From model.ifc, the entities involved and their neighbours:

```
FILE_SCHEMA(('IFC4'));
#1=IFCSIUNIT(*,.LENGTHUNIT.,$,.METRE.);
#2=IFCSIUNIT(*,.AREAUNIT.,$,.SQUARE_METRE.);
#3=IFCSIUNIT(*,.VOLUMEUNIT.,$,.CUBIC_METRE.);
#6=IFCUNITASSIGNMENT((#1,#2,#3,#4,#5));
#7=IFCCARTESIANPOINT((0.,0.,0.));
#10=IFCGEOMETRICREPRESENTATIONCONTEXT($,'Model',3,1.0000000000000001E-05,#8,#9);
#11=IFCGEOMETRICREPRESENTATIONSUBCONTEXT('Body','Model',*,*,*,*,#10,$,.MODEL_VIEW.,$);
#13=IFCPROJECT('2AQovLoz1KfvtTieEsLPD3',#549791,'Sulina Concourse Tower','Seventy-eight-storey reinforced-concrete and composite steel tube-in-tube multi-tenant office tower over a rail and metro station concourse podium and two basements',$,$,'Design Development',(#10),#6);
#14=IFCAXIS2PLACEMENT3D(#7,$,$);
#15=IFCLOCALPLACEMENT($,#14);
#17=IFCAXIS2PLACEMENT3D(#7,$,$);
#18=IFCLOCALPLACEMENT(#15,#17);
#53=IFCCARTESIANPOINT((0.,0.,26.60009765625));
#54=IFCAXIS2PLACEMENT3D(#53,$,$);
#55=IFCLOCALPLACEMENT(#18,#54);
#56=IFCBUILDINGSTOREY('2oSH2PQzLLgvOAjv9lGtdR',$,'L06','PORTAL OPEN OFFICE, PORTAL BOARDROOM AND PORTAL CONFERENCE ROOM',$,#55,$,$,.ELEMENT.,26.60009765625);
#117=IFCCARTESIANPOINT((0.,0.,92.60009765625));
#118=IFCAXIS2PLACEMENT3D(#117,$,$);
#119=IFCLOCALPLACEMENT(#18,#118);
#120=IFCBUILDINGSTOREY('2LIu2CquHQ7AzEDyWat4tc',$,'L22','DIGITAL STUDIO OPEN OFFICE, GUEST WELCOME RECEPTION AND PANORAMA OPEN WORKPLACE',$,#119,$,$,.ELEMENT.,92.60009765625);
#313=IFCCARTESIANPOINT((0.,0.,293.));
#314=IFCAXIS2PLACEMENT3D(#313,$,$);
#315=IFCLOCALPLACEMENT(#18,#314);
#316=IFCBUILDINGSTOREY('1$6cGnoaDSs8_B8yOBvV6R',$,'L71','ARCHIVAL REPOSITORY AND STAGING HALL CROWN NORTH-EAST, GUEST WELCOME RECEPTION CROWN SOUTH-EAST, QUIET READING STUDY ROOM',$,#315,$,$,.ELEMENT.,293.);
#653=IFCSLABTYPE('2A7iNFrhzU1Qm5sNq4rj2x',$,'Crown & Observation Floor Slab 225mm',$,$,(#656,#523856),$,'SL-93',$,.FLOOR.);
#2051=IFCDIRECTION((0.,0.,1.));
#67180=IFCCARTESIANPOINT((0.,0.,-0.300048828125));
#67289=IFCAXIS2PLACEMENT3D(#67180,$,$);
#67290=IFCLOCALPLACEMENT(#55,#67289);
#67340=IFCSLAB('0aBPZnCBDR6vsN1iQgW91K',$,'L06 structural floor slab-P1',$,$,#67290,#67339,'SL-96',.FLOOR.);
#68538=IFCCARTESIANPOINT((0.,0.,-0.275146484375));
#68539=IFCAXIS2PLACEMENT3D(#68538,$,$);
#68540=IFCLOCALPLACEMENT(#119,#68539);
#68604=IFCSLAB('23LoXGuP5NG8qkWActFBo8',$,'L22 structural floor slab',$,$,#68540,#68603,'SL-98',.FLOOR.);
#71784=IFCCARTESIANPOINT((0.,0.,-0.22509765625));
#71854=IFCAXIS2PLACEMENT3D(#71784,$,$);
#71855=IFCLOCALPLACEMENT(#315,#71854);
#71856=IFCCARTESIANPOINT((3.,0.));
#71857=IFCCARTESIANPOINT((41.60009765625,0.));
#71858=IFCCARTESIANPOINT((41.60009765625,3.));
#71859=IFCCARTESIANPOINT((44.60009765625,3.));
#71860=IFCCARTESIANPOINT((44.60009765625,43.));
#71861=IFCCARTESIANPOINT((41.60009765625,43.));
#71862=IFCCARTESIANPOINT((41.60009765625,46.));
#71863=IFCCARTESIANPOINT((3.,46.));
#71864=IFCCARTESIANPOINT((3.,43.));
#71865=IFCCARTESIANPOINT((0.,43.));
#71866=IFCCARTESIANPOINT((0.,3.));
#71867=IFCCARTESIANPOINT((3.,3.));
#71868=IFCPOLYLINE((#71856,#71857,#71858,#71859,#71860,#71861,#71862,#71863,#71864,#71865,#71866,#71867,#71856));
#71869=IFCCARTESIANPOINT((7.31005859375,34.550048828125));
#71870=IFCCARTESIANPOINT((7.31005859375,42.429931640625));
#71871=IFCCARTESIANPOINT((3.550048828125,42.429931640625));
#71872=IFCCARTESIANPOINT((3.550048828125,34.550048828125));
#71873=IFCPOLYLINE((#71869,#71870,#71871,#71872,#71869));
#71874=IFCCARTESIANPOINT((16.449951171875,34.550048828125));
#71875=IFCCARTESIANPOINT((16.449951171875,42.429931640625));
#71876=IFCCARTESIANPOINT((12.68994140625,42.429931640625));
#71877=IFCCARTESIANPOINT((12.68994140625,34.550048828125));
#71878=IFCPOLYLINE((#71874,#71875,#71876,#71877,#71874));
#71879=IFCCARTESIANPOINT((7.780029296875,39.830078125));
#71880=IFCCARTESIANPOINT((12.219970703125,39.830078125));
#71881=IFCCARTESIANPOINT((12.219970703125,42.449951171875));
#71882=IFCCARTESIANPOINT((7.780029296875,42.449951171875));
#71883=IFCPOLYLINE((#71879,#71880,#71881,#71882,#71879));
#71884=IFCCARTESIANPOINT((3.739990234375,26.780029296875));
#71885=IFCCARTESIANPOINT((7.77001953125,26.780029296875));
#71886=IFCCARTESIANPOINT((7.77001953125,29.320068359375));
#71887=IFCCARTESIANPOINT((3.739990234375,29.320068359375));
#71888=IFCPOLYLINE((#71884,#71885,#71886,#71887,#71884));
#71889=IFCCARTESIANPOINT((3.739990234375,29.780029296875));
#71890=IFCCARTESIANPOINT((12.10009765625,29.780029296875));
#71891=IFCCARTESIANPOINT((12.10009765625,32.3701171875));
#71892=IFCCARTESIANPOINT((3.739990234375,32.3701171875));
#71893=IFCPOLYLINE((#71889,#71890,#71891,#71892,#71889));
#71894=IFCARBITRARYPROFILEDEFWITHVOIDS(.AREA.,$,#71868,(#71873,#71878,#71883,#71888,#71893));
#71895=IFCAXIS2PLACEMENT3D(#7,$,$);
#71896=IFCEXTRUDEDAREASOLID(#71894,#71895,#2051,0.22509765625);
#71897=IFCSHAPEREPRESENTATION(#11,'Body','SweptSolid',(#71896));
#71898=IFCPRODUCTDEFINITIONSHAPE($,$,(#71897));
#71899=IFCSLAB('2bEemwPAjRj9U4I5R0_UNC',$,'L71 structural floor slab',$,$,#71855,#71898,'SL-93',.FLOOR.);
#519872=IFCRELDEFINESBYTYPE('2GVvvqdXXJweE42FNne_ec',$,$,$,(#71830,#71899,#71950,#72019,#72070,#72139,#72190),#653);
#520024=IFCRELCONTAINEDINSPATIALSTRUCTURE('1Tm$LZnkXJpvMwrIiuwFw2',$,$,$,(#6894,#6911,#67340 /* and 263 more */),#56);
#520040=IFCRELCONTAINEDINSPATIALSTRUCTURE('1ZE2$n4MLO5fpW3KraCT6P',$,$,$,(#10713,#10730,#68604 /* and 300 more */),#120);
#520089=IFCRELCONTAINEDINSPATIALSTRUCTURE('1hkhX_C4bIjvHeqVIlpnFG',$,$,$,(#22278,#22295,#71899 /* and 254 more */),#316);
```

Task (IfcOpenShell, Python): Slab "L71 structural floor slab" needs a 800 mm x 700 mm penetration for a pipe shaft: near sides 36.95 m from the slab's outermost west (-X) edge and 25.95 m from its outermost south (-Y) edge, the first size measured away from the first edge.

```python
import numpy as np
import ifcopenshell
import ifcopenshell.api.feature
import ifcopenshell.api.geometry
import ifcopenshell.api.root
import ifcopenshell.geom
import ifcopenshell.util.placement
import ifcopenshell.util.representation
import ifcopenshell.util.shape
import ifcopenshell.util.unit

model = ifcopenshell.open("model.ifc")
unit_scale = ifcopenshell.util.unit.calculate_unit_scale(model)
settings = ifcopenshell.geom.settings()


def volume(element):
    """Net volume in cubic metres, openings subtracted."""
    shape = ifcopenshell.geom.create_shape(settings, element)
    return ifcopenshell.util.shape.get_volume(shape.geometry)


slab = model.by_guid("2bEemwPAjRj9U4I5R0_UNC")
before = volume(slab)

# Extent in the slab's own axes, in metres. The edges named are its -X and -Y sides.
slab_shape = ifcopenshell.geom.create_shape(settings, slab)
vertices = ifcopenshell.util.shape.get_vertices(slab_shape.geometry)
x_min, y_min, bottom = vertices.min(axis=0)
top = vertices[:, 2].max()

opening = ifcopenshell.api.root.create_entity(model, ifc_class="IfcOpeningElement", name="Pipe shaft opening", predefined_type="OPENING")
context = ifcopenshell.util.representation.get_context(model, "Model", "Body", "MODEL_VIEW")
width, depth = 0.8, 0.7
outline = [(0.0, 0.0), (width, 0.0), (width, depth), (0.0, depth), (0.0, 0.0)]
# Overshoot both faces by 50 mm so the cut is clean.
shape = ifcopenshell.api.geometry.add_slab_representation(
    model, context=context, depth=top - bottom + 0.1, polyline=outline
)
ifcopenshell.api.geometry.assign_representation(model, product=opening, representation=shape)

matrix = ifcopenshell.util.placement.get_local_placement(slab.ObjectPlacement)
matrix[:, 3] = matrix @ np.append(np.array([x_min + 36.95, y_min + 25.95, bottom - 0.05]) / unit_scale, 1.0)
ifcopenshell.api.geometry.edit_object_placement(model, product=opening, matrix=matrix, is_si=False)
ifcopenshell.api.feature.add_feature(model, feature=opening, element=slab)

after = volume(slab)

print(f"slab volume {before:.3f} -> {after:.3f} m3")

model.write("model_rev.ifc")
```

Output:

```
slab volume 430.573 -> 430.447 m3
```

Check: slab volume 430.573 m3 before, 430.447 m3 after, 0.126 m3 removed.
